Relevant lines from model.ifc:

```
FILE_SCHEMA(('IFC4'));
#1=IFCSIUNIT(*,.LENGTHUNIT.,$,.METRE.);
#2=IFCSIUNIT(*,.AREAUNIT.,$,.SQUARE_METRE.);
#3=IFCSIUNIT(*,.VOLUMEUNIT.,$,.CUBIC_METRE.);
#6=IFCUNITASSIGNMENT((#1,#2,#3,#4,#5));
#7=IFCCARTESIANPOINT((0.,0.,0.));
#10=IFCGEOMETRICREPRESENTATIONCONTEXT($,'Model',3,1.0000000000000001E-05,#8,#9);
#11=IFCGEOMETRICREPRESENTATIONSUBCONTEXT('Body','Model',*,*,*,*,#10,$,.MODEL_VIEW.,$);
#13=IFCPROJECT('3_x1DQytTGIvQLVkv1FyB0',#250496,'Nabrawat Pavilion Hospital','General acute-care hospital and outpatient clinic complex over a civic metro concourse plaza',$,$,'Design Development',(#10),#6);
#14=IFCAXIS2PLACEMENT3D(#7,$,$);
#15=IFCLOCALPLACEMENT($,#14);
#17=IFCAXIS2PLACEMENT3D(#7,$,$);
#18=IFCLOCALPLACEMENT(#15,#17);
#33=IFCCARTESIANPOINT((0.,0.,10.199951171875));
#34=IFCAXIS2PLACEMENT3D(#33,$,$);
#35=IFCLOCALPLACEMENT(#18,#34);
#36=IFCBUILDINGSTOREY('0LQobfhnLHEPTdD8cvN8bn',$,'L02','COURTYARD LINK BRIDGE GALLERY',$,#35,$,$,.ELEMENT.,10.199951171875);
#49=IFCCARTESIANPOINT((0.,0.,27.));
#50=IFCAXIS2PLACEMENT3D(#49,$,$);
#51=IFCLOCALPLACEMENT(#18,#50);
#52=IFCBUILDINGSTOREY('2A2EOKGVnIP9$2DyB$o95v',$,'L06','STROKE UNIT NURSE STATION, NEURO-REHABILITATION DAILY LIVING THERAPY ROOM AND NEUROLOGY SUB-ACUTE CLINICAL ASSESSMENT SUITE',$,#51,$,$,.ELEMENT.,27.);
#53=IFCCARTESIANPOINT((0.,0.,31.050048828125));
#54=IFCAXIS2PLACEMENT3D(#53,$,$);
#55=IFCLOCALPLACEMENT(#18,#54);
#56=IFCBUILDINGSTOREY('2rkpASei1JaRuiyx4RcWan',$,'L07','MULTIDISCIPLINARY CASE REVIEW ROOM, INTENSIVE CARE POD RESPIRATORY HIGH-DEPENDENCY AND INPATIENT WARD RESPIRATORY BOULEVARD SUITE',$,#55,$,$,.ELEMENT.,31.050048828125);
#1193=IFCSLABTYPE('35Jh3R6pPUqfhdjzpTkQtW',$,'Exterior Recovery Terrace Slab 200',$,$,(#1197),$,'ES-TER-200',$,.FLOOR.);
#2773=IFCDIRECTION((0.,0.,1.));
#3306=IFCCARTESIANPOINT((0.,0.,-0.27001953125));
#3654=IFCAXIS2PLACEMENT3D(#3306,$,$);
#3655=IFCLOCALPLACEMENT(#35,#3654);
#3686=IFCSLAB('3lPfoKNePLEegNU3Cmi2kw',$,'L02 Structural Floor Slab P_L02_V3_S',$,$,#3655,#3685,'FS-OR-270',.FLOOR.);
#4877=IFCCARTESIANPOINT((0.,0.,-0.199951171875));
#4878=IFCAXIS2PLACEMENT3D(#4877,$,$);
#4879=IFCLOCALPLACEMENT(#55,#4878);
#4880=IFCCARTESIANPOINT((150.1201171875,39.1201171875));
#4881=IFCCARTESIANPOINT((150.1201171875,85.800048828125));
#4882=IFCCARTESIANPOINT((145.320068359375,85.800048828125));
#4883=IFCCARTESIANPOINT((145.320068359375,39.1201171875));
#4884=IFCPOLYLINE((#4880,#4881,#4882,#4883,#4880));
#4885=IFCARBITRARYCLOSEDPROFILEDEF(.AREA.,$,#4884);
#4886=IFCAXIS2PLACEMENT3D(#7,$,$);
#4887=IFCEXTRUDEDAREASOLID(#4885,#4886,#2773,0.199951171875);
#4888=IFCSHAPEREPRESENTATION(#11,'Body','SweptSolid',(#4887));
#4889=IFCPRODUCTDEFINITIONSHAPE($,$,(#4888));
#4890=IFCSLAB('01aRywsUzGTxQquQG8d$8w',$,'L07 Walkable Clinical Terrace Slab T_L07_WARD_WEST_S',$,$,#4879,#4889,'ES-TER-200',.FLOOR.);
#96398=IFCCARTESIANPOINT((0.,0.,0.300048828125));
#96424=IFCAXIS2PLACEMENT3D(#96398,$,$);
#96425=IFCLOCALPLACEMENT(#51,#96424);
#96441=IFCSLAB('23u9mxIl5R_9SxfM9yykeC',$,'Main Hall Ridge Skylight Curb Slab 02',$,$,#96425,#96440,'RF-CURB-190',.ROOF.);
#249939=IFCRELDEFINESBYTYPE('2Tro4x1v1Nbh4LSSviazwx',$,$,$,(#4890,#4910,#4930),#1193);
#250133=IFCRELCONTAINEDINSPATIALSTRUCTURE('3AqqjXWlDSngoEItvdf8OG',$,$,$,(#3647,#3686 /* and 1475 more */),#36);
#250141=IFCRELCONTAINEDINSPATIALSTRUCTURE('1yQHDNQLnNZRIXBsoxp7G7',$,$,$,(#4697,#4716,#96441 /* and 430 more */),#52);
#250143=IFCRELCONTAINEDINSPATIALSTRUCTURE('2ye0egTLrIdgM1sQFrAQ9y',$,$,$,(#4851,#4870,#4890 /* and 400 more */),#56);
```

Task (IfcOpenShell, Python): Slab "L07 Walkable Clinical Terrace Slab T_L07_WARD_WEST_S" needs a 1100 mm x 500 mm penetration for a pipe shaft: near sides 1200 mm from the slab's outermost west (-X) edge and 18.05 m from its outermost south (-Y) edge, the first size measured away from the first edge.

```python
import numpy as np
import ifcopenshell
import ifcopenshell.api.feature
import ifcopenshell.api.geometry
import ifcopenshell.api.root
import ifcopenshell.geom
import ifcopenshell.util.placement
import ifcopenshell.util.representation
import ifcopenshell.util.shape
import ifcopenshell.util.unit

model = ifcopenshell.open("model.ifc")
unit_scale = ifcopenshell.util.unit.calculate_unit_scale(model)
settings = ifcopenshell.geom.settings()


def volume(element):
    """Net volume in cubic metres, openings subtracted."""
    shape = ifcopenshell.geom.create_shape(settings, element)
    return ifcopenshell.util.shape.get_volume(shape.geometry)


slab = model.by_guid("01aRywsUzGTxQquQG8d$8w")
before = volume(slab)

# Extent in the slab's own axes, in metres. The edges named are its -X and -Y sides.
slab_shape = ifcopenshell.geom.create_shape(settings, slab)
vertices = ifcopenshell.util.shape.get_vertices(slab_shape.geometry)
x_min, y_min, bottom = vertices.min(axis=0)
top = vertices[:, 2].max()

opening = ifcopenshell.api.root.create_entity(model, ifc_class="IfcOpeningElement", name="Pipe shaft opening", predefined_type="OPENING")
context = ifcopenshell.util.representation.get_context(model, "Model", "Body", "MODEL_VIEW")
width, depth = 1.1, 0.5
outline = [(0.0, 0.0), (width, 0.0), (width, depth), (0.0, depth), (0.0, 0.0)]
# Overshoot both faces by 50 mm so the cut is clean.
shape = ifcopenshell.api.geometry.add_slab_representation(
    model, context=context, depth=top - bottom + 0.1, polyline=outline
)
ifcopenshell.api.geometry.assign_representation(model, product=opening, representation=shape)

matrix = ifcopenshell.util.placement.get_local_placement(slab.ObjectPlacement)
matrix[:, 3] = matrix @ np.append(np.array([x_min + 1.2, y_min + 18.05, bottom - 0.05]) / unit_scale, 1.0)
ifcopenshell.api.geometry.edit_object_placement(model, product=opening, matrix=matrix, is_si=False)
ifcopenshell.api.feature.add_feature(model, feature=opening, element=slab)

after = volume(slab)

print(f"slab volume {before:.3f} -> {after:.3f} m3")

model.write("model_v2.ifc")
```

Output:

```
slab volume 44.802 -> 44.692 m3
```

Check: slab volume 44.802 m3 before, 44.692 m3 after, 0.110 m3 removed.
